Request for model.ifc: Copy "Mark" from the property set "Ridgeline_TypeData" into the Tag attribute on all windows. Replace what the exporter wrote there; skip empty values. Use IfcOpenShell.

First a look at what the model holds.

```python
import ifcopenshell
import ifcopenshell.util.element

model = ifcopenshell.open("model.ifc")
print(model.schema)
windows = model.by_type("IfcWindow")
print(len(windows), "windows")
for e in windows[:8]:
    source = ifcopenshell.util.element.get_pset(e, "Ridgeline_TypeData", "Mark")
    target = e.Tag
    print(e.id(), repr(source), repr(target), sep=" | ")
```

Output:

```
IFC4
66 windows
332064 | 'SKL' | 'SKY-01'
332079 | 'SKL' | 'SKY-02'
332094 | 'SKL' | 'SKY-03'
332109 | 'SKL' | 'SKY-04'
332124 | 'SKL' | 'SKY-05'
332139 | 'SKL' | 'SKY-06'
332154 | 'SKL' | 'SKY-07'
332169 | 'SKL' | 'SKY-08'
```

```python
import ifcopenshell
import ifcopenshell.util.element

model = ifcopenshell.open("model.ifc")

count = 0
for e in model.by_type("IfcWindow"):
    value = ifcopenshell.util.element.get_pset(e, "Ridgeline_TypeData", "Mark")
    current = e.Tag
    if not value or not value.strip() or current == value:
        continue
    e.Tag = value
    count += 1

print(count, "windows updated")

model.write("model-out.ifc")
```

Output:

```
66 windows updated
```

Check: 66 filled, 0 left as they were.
